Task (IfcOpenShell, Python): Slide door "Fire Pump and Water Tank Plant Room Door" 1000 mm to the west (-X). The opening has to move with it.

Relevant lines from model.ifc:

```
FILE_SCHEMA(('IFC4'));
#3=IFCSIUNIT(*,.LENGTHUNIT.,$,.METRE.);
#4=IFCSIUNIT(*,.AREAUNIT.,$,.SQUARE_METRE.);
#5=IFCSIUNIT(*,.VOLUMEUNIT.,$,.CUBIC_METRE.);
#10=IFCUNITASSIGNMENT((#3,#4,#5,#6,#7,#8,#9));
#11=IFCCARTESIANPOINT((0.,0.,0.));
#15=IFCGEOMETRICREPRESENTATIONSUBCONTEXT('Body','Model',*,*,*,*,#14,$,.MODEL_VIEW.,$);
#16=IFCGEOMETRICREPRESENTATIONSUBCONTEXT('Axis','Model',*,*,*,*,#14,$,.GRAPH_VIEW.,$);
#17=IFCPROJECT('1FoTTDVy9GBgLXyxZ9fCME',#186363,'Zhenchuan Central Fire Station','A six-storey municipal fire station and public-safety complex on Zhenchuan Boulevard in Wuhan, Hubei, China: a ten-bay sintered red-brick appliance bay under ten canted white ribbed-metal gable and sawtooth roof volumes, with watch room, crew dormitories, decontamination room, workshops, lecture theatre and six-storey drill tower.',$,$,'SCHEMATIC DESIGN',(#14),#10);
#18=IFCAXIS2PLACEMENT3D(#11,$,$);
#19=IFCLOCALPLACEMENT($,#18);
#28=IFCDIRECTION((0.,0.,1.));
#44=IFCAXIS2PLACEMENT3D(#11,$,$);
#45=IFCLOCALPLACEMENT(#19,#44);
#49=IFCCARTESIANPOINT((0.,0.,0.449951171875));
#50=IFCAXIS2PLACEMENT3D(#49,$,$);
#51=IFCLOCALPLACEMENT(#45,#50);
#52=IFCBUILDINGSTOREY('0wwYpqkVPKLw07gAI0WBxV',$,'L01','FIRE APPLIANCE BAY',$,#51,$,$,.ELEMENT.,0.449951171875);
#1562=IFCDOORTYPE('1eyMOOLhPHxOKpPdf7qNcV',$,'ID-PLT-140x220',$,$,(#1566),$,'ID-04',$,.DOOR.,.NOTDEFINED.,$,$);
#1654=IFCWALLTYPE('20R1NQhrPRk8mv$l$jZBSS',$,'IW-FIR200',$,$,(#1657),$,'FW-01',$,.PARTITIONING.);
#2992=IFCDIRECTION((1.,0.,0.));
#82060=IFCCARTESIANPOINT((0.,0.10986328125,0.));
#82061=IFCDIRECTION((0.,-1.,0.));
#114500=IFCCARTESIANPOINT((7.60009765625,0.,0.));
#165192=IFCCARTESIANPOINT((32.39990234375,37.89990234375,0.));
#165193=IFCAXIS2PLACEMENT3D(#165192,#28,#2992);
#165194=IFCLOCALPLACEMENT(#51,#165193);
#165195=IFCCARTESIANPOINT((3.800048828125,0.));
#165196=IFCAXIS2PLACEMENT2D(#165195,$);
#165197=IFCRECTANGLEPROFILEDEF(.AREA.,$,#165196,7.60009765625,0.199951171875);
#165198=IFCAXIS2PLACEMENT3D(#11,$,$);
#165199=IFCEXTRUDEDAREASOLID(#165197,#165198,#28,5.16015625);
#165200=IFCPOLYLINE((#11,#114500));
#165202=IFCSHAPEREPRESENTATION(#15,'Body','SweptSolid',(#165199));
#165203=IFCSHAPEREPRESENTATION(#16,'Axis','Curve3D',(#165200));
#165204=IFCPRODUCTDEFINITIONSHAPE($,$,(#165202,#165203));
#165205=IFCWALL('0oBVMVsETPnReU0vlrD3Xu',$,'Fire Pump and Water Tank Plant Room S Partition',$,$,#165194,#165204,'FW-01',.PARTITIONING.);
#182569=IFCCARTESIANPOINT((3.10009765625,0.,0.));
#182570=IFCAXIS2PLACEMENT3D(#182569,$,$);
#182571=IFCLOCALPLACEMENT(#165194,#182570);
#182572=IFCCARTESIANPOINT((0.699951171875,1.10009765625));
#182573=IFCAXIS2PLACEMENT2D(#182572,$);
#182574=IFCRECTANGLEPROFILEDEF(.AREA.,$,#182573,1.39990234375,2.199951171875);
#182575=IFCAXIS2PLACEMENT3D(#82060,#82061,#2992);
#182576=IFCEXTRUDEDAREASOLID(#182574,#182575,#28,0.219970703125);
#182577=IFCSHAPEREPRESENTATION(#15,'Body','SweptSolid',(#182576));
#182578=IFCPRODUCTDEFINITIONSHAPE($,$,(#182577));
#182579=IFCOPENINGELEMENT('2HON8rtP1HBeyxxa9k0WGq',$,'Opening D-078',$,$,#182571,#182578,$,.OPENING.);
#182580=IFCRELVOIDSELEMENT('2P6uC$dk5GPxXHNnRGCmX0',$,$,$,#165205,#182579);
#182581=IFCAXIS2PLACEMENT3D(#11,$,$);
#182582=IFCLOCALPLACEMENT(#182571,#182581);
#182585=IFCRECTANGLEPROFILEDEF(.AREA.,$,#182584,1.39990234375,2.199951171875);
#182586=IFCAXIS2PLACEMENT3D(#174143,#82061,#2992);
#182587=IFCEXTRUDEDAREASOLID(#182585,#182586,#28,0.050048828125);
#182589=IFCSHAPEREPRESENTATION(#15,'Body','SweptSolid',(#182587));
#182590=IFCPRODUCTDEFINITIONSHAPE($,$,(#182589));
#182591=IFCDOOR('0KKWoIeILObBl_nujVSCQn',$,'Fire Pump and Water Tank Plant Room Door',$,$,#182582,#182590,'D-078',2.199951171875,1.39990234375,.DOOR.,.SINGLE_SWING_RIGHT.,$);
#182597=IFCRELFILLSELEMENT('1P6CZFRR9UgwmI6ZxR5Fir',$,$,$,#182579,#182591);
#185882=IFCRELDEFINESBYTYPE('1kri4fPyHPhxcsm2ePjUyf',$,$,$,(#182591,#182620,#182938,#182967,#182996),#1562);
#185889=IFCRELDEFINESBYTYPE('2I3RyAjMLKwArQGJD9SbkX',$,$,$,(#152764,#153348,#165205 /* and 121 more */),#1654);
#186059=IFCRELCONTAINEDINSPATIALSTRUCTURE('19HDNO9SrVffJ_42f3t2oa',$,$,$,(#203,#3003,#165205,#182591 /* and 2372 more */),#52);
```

```python
import ifcopenshell
import ifcopenshell.api.geometry
import ifcopenshell.util.placement

model = ifcopenshell.open("model.ifc")

door = model.by_guid("0KKWoIeILObBl_nujVSCQn")
opening = door.FillsVoids[0].RelatingOpeningElement
wall = opening.VoidsElements[0].RelatingBuildingElement

wall_matrix = ifcopenshell.util.placement.get_local_placement(wall.ObjectPlacement)
shift = wall_matrix[:3, 0] * -1.0
before = ifcopenshell.util.placement.get_local_placement(door.ObjectPlacement)[:3, 3].copy()

# The door is placed relative to its opening, so it follows when the opening moves.
matrix = ifcopenshell.util.placement.get_local_placement(opening.ObjectPlacement)
matrix[:3, 3] += shift
ifcopenshell.api.geometry.edit_object_placement(
    model, product=opening, matrix=matrix, is_si=False, should_transform_children=True
)

after = ifcopenshell.util.placement.get_local_placement(door.ObjectPlacement)[:3, 3]
print("door moved by", (after - before).round(3) + 0.0)

model.write("model_edited.ifc")
```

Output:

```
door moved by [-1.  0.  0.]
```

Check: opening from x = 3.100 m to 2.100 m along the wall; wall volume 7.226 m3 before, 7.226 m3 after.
